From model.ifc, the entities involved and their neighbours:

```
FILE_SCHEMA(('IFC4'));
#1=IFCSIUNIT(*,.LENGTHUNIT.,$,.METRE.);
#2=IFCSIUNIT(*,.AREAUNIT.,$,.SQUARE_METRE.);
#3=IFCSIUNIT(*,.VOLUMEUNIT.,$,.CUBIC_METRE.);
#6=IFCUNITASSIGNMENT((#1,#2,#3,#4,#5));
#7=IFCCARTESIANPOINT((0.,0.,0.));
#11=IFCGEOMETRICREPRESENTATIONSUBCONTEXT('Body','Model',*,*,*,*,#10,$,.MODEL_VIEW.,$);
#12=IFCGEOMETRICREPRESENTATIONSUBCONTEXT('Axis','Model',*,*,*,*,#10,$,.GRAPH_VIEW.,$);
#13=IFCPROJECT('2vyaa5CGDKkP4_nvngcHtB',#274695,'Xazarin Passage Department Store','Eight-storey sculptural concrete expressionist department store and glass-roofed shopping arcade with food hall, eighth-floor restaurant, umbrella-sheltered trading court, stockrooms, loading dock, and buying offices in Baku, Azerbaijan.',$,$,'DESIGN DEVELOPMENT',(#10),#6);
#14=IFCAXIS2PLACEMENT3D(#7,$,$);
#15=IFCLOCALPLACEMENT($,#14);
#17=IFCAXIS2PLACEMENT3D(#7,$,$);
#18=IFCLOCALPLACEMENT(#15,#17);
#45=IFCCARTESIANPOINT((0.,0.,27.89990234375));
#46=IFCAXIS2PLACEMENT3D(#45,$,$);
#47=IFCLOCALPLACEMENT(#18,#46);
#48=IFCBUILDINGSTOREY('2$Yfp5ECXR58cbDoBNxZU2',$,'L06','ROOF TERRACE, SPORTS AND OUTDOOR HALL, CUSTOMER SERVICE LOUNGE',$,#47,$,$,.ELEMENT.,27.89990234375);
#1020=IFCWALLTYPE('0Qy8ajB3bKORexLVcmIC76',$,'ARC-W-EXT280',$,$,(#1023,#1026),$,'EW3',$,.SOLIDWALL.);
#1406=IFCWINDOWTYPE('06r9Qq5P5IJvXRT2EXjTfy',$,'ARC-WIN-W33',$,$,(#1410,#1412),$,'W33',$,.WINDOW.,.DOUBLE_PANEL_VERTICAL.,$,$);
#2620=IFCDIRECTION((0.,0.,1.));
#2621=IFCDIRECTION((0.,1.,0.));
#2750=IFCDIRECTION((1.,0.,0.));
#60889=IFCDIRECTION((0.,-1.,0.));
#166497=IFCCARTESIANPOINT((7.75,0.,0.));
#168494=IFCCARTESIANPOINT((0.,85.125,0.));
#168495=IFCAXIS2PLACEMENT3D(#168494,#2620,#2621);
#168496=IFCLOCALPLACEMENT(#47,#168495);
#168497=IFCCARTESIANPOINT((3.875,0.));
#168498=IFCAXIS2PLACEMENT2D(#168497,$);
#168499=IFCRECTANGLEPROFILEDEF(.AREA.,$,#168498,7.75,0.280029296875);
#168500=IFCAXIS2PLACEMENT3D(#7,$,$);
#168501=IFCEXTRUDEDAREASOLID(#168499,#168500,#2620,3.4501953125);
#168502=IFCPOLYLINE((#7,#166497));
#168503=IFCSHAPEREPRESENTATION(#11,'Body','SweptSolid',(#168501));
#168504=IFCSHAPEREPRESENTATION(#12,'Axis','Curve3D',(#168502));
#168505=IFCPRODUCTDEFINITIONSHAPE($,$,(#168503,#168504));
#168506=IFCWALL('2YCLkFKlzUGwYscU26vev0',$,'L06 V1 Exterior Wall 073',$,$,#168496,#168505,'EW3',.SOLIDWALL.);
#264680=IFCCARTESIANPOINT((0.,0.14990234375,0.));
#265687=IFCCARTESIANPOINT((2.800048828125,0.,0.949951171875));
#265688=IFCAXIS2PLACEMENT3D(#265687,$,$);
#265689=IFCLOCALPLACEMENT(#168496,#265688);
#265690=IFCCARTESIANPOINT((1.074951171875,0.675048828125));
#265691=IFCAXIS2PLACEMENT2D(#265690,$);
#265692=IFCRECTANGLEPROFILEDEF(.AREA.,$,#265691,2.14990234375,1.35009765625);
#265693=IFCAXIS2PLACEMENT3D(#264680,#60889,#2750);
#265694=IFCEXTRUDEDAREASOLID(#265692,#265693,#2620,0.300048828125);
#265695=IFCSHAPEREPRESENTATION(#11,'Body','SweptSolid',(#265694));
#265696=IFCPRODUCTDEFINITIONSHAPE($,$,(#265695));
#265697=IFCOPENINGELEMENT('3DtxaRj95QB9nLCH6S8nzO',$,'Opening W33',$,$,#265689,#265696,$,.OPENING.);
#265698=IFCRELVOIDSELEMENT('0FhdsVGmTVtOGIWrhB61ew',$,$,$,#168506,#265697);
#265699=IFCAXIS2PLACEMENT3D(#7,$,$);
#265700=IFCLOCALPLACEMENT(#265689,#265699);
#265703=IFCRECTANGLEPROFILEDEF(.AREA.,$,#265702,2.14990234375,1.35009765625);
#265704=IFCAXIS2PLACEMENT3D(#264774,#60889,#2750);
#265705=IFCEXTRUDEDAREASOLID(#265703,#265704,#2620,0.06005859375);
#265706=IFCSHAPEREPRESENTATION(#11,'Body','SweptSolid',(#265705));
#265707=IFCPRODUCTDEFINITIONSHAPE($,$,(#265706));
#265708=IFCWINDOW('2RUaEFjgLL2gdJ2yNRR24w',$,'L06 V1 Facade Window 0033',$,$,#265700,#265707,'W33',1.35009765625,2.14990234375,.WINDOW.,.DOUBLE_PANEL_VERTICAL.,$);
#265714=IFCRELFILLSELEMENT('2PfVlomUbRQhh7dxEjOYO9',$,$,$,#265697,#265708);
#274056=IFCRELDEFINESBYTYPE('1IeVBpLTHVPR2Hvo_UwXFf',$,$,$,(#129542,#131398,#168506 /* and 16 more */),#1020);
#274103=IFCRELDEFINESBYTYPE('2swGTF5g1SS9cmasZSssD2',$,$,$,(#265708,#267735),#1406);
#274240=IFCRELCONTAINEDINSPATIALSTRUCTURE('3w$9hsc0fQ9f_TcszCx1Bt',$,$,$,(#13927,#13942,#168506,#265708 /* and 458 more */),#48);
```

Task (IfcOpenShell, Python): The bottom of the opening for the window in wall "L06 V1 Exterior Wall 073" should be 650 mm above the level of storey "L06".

```python
import numpy as np
import ifcopenshell
import ifcopenshell.api.geometry
import ifcopenshell.geom
import ifcopenshell.util.element
import ifcopenshell.util.placement
import ifcopenshell.util.shape
import ifcopenshell.util.unit

model = ifcopenshell.open("model.ifc")
unit_scale = ifcopenshell.util.unit.calculate_unit_scale(model)

window = model.by_id(265708)
opening = window.FillsVoids[0].RelatingOpeningElement
storey = ifcopenshell.util.element.get_container(window, ifc_class="IfcBuildingStorey")
level = ifcopenshell.util.placement.get_local_placement(storey.ObjectPlacement)[2, 3]

# The opening's origin need not be at the sill, so measure its lowest point.
shape = ifcopenshell.geom.create_shape(ifcopenshell.geom.settings(), opening)
bottom = ifcopenshell.util.shape.get_shape_bottom_elevation(shape, shape.geometry) / unit_scale
dz = level + 0.65 / unit_scale - bottom

shift = np.array([0.0, 0.0, dz])
# The window is placed relative to its opening, so it follows when the opening moves.
matrix = ifcopenshell.util.placement.get_local_placement(opening.ObjectPlacement)
matrix[:3, 3] += shift
ifcopenshell.api.geometry.edit_object_placement(
    model, product=opening, matrix=matrix, is_si=False, should_transform_children=True
)

print(f"moved by {dz * unit_scale:+.3f} m")

model.write("model_updated.ifc")
```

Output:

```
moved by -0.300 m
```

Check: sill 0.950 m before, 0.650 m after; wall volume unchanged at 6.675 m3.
